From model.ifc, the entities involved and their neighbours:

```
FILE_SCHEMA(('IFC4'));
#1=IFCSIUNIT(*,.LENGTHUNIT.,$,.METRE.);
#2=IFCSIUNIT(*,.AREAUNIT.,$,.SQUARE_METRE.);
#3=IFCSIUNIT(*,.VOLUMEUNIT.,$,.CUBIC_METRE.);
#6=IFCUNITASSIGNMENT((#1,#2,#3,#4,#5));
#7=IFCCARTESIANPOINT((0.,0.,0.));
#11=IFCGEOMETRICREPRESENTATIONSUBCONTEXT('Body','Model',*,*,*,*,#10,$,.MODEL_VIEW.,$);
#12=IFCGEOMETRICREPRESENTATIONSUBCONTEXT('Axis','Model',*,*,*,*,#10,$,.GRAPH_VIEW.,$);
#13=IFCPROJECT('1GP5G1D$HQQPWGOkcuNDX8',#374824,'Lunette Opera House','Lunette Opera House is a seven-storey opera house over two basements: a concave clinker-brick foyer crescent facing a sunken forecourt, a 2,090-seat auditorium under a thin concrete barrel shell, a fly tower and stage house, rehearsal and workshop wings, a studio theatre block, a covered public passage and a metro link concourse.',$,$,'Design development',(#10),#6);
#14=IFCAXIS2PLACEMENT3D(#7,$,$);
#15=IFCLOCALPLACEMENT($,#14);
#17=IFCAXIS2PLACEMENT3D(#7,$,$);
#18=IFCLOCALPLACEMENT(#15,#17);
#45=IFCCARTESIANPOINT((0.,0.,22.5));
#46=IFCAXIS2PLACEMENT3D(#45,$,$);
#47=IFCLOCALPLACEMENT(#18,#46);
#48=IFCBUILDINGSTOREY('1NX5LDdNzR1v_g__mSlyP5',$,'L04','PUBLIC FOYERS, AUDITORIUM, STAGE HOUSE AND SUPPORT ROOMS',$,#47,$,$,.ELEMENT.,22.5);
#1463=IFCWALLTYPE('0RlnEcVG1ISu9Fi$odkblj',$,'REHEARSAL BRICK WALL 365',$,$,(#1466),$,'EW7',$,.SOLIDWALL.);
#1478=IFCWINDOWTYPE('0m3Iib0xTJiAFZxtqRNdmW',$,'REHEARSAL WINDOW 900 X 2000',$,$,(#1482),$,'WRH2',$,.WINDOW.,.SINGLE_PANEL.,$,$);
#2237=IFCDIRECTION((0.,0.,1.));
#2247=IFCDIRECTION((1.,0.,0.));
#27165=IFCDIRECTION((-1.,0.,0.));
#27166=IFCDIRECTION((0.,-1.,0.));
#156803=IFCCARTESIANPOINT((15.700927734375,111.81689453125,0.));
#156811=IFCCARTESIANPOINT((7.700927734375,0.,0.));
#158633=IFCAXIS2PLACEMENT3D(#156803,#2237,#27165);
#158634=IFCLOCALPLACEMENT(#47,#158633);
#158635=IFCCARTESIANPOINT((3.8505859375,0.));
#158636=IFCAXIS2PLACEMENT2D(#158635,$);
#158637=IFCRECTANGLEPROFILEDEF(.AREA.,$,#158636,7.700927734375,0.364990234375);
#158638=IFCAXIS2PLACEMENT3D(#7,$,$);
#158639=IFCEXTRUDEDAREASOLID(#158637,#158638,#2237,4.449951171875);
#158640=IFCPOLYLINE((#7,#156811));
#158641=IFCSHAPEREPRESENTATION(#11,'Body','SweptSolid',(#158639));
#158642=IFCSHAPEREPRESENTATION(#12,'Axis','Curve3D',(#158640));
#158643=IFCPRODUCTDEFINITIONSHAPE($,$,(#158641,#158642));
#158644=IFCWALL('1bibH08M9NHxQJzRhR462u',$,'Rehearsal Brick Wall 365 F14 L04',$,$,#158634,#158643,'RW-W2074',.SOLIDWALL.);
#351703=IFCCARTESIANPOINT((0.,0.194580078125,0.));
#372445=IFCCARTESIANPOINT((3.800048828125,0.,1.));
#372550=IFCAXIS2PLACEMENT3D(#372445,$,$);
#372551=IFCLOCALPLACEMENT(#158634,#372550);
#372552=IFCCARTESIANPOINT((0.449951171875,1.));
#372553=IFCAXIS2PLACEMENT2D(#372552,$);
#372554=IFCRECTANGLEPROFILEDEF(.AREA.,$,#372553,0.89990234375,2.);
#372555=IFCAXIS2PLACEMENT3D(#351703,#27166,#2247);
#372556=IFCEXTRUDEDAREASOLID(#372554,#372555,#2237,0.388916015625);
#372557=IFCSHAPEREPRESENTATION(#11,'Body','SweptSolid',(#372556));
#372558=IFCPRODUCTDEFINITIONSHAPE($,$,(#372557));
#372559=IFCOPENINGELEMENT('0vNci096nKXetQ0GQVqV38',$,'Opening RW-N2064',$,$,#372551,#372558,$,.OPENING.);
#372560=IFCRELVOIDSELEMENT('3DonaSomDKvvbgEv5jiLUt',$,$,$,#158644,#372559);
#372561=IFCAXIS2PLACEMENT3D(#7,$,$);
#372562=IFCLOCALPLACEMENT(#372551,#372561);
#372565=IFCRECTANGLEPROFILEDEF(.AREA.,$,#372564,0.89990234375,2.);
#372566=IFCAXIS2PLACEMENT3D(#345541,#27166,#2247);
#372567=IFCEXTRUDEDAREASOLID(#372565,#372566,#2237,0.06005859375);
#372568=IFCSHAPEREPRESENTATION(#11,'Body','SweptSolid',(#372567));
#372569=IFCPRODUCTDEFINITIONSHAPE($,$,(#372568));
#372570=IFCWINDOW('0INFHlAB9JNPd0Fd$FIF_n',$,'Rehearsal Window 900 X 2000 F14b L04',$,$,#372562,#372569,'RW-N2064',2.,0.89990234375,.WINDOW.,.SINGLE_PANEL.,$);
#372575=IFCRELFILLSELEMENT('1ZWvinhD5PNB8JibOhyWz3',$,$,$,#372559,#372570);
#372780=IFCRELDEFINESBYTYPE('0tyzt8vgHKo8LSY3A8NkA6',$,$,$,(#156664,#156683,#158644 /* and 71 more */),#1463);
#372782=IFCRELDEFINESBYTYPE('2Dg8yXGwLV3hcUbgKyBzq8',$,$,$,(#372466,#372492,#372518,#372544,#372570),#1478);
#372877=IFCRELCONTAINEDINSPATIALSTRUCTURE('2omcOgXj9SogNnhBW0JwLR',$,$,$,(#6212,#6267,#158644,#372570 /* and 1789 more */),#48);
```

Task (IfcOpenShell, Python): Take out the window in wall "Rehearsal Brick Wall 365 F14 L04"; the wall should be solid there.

```python
import ifcopenshell
import ifcopenshell.api.feature
import ifcopenshell.api.root
import ifcopenshell.geom
import ifcopenshell.util.shape

model = ifcopenshell.open("model.ifc")
settings = ifcopenshell.geom.settings()


def volume(element):
    """Net volume in cubic metres, openings subtracted."""
    shape = ifcopenshell.geom.create_shape(settings, element)
    return ifcopenshell.util.shape.get_volume(shape.geometry)


window = model.by_guid("0INFHlAB9JNPd0Fd$FIF_n")
opening = window.FillsVoids[0].RelatingOpeningElement
wall = opening.VoidsElements[0].RelatingBuildingElement
before = volume(wall)

ifcopenshell.api.root.remove_product(model, product=window)
ifcopenshell.api.feature.remove_feature(model, feature=opening)

after = volume(wall)

print(f"wall volume {before:.3f} -> {after:.3f} m3")

model.write("model_rev.ifc")
```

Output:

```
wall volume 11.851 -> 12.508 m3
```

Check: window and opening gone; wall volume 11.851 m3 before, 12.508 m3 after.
